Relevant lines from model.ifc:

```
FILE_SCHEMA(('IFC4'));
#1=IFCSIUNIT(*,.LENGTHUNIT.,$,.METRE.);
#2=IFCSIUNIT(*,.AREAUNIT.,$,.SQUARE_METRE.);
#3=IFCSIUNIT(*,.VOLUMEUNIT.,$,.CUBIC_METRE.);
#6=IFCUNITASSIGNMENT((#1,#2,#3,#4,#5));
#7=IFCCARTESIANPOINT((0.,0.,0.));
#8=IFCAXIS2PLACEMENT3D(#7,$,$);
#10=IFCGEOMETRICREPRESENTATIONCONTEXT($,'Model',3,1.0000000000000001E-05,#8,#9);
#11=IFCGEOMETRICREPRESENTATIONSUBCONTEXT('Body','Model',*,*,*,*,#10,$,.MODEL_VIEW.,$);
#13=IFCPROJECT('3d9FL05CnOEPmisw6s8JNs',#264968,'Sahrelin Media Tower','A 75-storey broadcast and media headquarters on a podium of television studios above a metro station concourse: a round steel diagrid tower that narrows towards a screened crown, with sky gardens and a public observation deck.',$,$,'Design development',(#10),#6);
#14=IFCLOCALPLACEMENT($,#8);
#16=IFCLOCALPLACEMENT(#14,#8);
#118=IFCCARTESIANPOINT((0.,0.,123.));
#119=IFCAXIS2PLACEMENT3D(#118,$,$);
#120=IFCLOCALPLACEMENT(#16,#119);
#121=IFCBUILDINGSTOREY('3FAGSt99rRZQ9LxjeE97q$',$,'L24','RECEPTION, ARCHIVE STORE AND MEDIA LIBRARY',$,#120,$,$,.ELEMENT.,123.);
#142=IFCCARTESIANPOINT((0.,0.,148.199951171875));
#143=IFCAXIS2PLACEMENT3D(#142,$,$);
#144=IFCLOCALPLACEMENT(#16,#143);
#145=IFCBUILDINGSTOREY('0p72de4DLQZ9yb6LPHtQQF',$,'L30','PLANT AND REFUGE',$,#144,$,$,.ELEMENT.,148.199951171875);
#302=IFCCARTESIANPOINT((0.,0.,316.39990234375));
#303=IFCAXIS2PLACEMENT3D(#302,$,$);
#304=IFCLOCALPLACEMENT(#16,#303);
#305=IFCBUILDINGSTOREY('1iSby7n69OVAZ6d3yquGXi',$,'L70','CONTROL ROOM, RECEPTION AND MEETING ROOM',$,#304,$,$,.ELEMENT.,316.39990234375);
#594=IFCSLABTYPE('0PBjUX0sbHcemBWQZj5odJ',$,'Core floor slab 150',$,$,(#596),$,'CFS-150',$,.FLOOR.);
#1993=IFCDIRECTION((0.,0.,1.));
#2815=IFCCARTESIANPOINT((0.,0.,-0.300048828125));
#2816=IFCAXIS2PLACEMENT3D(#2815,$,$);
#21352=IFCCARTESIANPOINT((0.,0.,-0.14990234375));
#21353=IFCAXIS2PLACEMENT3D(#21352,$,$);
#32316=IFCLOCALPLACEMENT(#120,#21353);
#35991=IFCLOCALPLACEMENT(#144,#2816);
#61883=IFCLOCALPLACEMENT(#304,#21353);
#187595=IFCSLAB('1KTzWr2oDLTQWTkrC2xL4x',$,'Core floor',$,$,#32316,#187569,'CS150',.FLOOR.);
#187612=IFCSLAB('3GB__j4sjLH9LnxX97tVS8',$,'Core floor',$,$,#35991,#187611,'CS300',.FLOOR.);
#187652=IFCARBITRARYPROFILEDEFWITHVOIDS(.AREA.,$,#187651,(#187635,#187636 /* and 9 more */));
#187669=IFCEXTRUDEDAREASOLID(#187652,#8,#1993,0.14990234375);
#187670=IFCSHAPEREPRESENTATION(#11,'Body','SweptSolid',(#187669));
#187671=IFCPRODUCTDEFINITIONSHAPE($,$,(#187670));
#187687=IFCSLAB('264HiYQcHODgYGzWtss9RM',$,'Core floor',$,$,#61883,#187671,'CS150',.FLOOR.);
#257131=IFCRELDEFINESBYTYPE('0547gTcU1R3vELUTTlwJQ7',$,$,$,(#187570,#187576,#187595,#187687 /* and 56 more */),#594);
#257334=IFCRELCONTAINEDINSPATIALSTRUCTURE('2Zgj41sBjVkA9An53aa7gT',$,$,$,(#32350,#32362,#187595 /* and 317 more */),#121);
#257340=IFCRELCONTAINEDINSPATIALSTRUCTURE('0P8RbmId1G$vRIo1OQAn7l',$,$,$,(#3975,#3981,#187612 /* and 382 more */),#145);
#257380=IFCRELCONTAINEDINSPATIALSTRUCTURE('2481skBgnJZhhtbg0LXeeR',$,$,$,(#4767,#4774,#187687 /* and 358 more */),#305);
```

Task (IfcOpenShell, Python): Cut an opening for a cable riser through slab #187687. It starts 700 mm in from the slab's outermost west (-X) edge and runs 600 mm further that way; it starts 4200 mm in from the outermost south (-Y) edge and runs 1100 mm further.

```python
import numpy as np
import ifcopenshell
import ifcopenshell.api.feature
import ifcopenshell.api.geometry
import ifcopenshell.api.root
import ifcopenshell.geom
import ifcopenshell.util.placement
import ifcopenshell.util.representation
import ifcopenshell.util.shape
import ifcopenshell.util.unit

model = ifcopenshell.open("model.ifc")
unit_scale = ifcopenshell.util.unit.calculate_unit_scale(model)
settings = ifcopenshell.geom.settings()


def volume(element):
    """Net volume in cubic metres, openings subtracted."""
    shape = ifcopenshell.geom.create_shape(settings, element)
    return ifcopenshell.util.shape.get_volume(shape.geometry)


slab = model.by_guid("264HiYQcHODgYGzWtss9RM")
before = volume(slab)

# Extent in the slab's own axes, in metres. The edges named are its -X and -Y sides.
slab_shape = ifcopenshell.geom.create_shape(settings, slab)
vertices = ifcopenshell.util.shape.get_vertices(slab_shape.geometry)
x_min, y_min, bottom = vertices.min(axis=0)
top = vertices[:, 2].max()

opening = ifcopenshell.api.root.create_entity(model, ifc_class="IfcOpeningElement", name="Cable riser opening", predefined_type="OPENING")
context = ifcopenshell.util.representation.get_context(model, "Model", "Body", "MODEL_VIEW")
width, depth = 0.6, 1.1
outline = [(0.0, 0.0), (width, 0.0), (width, depth), (0.0, depth), (0.0, 0.0)]
# Overshoot both faces by 50 mm so the cut is clean.
shape = ifcopenshell.api.geometry.add_slab_representation(
    model, context=context, depth=top - bottom + 0.1, polyline=outline
)
ifcopenshell.api.geometry.assign_representation(model, product=opening, representation=shape)

matrix = ifcopenshell.util.placement.get_local_placement(slab.ObjectPlacement)
matrix[:, 3] = matrix @ np.append(np.array([x_min + 0.7, y_min + 4.2, bottom - 0.05]) / unit_scale, 1.0)
ifcopenshell.api.geometry.edit_object_placement(model, product=opening, matrix=matrix, is_si=False)
ifcopenshell.api.feature.add_feature(model, feature=opening, element=slab)

after = volume(slab)

print(f"slab volume {before:.3f} -> {after:.3f} m3")

model.write("model_v2.ifc")
```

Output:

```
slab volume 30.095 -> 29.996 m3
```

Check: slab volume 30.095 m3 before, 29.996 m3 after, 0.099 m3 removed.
